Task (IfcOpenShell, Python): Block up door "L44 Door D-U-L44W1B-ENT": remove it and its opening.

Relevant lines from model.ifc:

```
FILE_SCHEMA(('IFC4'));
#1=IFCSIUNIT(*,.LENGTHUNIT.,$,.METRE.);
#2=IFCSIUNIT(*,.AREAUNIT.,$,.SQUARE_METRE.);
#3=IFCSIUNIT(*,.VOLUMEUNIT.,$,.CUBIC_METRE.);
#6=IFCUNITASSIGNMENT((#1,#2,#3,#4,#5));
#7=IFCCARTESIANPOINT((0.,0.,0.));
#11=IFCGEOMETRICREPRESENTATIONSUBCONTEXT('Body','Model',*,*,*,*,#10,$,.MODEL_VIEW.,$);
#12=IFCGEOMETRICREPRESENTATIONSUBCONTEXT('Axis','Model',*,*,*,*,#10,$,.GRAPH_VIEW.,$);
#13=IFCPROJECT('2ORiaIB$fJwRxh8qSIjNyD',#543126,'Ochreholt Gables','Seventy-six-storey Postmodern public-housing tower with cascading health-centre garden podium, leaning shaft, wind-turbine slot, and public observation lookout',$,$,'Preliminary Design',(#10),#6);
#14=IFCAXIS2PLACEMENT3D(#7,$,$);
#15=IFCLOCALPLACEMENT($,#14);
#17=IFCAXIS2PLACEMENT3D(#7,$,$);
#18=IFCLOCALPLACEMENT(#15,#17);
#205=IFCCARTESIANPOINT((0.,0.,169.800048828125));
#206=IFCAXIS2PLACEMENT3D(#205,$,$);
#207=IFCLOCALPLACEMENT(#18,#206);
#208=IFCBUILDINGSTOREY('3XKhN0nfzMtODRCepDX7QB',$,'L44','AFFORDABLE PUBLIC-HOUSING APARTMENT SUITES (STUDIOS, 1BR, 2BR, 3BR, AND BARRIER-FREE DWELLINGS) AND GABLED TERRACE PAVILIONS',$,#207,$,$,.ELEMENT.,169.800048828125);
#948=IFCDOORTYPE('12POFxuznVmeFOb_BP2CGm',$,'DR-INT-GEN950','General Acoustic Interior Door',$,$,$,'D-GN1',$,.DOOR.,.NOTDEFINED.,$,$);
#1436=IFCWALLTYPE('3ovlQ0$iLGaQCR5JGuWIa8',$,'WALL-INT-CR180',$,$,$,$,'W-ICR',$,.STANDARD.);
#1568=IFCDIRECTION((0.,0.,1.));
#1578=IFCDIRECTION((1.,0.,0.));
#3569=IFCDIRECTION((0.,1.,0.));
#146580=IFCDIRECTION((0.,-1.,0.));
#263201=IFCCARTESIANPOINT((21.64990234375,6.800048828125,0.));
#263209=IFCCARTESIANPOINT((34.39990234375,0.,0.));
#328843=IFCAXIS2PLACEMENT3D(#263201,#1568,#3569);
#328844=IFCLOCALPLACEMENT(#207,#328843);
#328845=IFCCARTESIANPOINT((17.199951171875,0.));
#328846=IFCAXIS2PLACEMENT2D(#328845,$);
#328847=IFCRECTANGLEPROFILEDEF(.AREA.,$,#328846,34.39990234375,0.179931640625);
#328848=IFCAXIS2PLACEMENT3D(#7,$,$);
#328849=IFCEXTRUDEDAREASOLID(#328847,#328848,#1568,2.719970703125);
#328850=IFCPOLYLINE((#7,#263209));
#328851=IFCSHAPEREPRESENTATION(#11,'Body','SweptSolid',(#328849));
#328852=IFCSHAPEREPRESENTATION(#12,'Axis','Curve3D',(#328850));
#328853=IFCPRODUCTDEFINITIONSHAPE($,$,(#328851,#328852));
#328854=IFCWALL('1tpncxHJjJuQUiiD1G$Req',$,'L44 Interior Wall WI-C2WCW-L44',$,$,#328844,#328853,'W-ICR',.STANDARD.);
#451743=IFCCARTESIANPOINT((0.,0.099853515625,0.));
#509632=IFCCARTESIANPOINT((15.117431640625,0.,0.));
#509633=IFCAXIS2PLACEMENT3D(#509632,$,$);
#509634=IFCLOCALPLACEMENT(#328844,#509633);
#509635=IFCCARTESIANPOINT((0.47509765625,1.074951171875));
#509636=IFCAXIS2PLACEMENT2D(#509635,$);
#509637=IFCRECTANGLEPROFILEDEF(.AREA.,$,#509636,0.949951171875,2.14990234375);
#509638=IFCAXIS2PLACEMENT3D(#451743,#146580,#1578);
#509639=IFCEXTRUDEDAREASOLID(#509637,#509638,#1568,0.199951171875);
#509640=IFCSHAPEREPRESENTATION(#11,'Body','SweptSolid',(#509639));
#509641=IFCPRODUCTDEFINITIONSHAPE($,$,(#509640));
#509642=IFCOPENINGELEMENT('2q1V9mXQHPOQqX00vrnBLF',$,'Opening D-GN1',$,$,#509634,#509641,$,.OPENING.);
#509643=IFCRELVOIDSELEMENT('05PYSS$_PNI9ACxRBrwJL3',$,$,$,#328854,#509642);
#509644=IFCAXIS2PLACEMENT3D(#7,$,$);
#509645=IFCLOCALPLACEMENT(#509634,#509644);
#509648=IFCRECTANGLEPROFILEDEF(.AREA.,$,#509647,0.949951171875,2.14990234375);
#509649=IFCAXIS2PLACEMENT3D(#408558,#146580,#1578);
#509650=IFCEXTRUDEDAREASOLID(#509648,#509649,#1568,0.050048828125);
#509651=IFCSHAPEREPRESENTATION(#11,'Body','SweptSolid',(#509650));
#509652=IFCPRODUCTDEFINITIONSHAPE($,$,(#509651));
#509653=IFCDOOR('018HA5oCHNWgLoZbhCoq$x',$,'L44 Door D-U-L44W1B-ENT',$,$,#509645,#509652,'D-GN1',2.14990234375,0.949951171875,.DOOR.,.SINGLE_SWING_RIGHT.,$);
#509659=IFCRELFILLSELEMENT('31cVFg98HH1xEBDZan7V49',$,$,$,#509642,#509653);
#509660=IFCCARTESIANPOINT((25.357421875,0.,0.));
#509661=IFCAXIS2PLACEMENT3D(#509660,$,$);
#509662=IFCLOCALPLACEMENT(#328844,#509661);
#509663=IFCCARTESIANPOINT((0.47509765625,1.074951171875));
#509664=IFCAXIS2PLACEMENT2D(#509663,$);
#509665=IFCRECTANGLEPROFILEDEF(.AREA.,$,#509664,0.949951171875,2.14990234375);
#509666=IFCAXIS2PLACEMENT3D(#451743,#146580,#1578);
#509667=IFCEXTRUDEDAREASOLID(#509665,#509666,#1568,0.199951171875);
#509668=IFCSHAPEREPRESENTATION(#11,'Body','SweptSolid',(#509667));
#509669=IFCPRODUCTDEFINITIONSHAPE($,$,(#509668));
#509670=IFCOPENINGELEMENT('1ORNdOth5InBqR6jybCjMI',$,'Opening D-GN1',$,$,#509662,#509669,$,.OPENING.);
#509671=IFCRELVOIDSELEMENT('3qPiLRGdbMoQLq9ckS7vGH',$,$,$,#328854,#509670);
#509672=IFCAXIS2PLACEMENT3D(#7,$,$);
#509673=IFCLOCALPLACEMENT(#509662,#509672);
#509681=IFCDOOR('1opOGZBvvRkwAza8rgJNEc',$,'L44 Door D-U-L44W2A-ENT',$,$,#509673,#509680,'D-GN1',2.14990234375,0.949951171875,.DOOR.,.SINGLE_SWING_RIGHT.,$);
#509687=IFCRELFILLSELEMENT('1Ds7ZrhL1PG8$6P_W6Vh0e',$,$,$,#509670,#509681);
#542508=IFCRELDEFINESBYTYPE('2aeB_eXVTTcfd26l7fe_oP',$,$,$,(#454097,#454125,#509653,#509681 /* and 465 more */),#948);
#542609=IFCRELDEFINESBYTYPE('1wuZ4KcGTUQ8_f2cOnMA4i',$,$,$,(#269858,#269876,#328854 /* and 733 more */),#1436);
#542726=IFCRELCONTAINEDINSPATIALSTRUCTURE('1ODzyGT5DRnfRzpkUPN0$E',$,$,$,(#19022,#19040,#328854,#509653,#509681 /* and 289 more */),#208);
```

```python
import ifcopenshell
import ifcopenshell.api.feature
import ifcopenshell.api.root
import ifcopenshell.geom
import ifcopenshell.util.shape

model = ifcopenshell.open("model.ifc")
settings = ifcopenshell.geom.settings()


def volume(element):
    """Net volume in cubic metres, openings subtracted."""
    shape = ifcopenshell.geom.create_shape(settings, element)
    return ifcopenshell.util.shape.get_volume(shape.geometry)


door = model.by_guid("018HA5oCHNWgLoZbhCoq$x")
opening = door.FillsVoids[0].RelatingOpeningElement
wall = opening.VoidsElements[0].RelatingBuildingElement
before = volume(wall)

ifcopenshell.api.root.remove_product(model, product=door)
ifcopenshell.api.feature.remove_feature(model, feature=opening)

after = volume(wall)

print(f"wall volume {before:.3f} -> {after:.3f} m3")

model.write("model_edited.ifc")
```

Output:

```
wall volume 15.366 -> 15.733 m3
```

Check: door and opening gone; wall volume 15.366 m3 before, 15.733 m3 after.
